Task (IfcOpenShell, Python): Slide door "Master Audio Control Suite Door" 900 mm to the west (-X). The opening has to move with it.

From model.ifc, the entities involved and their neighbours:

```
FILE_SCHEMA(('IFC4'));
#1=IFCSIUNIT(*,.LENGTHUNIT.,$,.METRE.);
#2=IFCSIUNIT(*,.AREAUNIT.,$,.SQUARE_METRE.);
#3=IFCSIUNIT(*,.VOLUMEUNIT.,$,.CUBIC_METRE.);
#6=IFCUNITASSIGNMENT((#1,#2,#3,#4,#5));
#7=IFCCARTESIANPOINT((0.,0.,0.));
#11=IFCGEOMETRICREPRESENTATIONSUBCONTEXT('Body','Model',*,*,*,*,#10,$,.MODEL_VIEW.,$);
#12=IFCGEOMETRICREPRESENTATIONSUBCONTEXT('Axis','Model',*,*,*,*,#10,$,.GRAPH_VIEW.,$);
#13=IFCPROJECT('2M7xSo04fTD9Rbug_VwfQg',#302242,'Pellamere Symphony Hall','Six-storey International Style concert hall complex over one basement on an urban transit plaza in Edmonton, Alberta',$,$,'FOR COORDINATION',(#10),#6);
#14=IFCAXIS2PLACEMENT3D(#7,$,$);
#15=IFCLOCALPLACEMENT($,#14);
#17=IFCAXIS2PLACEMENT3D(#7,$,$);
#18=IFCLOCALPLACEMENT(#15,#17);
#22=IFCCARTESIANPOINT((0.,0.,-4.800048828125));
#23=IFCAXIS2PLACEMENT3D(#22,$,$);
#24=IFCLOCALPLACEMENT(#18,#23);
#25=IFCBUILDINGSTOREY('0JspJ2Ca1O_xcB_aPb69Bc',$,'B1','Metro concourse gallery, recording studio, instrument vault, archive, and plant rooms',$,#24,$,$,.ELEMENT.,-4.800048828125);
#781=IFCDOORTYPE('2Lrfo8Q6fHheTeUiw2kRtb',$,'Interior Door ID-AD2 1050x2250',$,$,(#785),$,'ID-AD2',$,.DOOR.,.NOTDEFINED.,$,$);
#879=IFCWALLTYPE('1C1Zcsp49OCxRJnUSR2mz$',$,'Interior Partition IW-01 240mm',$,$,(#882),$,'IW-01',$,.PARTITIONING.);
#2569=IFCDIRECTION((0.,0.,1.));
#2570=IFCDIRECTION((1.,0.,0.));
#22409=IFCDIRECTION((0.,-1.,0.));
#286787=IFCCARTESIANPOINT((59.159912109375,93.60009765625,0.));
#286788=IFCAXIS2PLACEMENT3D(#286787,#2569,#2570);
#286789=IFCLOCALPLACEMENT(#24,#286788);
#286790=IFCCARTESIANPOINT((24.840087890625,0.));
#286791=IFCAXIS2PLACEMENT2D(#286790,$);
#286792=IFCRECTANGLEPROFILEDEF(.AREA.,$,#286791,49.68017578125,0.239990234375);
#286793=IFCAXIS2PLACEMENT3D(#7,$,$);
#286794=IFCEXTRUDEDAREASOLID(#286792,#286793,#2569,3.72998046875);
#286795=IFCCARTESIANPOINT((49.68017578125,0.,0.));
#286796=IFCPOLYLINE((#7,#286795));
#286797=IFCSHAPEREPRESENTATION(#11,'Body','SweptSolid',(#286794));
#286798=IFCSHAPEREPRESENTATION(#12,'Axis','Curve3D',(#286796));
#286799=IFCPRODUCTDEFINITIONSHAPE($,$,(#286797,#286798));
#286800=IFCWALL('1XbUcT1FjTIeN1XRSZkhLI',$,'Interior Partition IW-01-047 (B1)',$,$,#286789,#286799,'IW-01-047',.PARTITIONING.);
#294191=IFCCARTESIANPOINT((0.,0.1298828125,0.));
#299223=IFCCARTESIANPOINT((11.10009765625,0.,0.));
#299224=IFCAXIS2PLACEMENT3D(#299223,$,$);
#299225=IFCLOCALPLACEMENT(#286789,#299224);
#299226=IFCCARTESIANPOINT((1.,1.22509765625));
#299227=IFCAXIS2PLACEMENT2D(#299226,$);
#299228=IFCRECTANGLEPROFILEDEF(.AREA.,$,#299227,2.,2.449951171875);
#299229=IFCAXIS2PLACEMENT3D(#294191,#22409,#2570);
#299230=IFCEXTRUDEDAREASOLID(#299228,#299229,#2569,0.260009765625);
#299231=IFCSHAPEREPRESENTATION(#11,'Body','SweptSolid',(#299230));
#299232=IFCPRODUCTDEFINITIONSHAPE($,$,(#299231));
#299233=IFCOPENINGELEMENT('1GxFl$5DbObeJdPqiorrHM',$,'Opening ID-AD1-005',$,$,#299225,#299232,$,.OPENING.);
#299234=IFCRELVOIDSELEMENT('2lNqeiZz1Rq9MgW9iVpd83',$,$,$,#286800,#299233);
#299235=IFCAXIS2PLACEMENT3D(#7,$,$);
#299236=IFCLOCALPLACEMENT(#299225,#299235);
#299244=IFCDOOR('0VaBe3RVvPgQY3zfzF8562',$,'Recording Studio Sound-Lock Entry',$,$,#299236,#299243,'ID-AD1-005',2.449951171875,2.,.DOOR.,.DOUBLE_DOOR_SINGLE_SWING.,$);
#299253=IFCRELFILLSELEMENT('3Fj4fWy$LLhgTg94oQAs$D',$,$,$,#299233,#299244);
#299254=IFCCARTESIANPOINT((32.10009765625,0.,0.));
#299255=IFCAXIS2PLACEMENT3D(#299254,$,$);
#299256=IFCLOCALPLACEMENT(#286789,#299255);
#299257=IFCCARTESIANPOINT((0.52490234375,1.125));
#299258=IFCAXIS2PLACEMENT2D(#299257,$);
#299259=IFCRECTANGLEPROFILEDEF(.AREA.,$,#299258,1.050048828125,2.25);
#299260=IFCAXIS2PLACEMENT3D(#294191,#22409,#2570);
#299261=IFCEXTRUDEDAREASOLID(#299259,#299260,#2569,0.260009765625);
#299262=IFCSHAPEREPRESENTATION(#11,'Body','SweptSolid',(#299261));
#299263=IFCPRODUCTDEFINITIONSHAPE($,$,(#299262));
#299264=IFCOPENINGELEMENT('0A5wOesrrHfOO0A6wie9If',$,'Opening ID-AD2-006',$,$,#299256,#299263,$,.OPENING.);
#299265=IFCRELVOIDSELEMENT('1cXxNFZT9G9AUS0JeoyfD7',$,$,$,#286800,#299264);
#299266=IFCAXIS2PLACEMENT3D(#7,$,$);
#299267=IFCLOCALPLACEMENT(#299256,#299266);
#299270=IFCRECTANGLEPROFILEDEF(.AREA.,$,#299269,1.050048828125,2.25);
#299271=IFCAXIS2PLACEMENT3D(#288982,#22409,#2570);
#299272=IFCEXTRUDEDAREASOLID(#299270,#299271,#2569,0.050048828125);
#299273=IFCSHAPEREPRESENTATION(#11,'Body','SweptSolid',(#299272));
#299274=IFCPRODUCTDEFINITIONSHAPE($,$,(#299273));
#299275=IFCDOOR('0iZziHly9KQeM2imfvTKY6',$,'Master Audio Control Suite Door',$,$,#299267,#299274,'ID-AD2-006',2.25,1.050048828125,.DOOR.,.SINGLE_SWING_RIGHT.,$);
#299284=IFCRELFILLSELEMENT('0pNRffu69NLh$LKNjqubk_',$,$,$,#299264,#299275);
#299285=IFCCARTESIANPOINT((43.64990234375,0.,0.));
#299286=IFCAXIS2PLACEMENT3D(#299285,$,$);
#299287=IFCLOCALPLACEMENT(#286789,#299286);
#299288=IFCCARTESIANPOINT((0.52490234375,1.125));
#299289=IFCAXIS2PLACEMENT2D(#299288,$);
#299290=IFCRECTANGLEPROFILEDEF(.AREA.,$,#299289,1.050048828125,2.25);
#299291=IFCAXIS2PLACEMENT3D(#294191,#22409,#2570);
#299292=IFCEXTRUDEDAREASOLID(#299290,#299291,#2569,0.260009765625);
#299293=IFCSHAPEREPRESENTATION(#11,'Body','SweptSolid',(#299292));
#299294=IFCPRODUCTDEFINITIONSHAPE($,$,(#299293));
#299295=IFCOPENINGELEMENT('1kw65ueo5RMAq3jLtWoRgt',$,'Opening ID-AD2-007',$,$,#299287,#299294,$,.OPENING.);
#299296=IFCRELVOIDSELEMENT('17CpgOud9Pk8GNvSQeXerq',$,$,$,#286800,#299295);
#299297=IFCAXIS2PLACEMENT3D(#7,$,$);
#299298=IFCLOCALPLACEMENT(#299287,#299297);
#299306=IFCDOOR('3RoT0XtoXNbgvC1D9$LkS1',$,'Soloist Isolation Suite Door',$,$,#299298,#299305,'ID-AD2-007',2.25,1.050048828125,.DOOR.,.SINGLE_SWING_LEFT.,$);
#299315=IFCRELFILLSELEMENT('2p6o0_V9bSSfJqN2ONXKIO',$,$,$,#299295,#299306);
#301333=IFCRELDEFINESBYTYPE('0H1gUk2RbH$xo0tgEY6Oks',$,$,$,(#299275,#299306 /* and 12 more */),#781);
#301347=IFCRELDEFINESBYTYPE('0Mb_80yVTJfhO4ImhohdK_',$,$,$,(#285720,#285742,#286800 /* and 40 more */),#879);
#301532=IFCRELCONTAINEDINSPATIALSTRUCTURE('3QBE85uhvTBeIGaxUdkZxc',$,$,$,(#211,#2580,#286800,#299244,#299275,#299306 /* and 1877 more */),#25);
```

```python
import ifcopenshell
import ifcopenshell.api.geometry
import ifcopenshell.util.placement

model = ifcopenshell.open("model.ifc")

door = model.by_guid("0iZziHly9KQeM2imfvTKY6")
opening = door.FillsVoids[0].RelatingOpeningElement
wall = opening.VoidsElements[0].RelatingBuildingElement

wall_matrix = ifcopenshell.util.placement.get_local_placement(wall.ObjectPlacement)
shift = wall_matrix[:3, 0] * -0.9
before = ifcopenshell.util.placement.get_local_placement(door.ObjectPlacement)[:3, 3].copy()

# The door is placed relative to its opening, so it follows when the opening moves.
matrix = ifcopenshell.util.placement.get_local_placement(opening.ObjectPlacement)
matrix[:3, 3] += shift
ifcopenshell.api.geometry.edit_object_placement(
    model, product=opening, matrix=matrix, is_si=False, should_transform_children=True
)

after = ifcopenshell.util.placement.get_local_placement(door.ObjectPlacement)[:3, 3]
print("door moved by", (after - before).round(3) + 0.0)

model.write("model_rev.ifc")
```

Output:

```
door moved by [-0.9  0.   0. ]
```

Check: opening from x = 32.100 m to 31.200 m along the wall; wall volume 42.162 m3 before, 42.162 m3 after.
